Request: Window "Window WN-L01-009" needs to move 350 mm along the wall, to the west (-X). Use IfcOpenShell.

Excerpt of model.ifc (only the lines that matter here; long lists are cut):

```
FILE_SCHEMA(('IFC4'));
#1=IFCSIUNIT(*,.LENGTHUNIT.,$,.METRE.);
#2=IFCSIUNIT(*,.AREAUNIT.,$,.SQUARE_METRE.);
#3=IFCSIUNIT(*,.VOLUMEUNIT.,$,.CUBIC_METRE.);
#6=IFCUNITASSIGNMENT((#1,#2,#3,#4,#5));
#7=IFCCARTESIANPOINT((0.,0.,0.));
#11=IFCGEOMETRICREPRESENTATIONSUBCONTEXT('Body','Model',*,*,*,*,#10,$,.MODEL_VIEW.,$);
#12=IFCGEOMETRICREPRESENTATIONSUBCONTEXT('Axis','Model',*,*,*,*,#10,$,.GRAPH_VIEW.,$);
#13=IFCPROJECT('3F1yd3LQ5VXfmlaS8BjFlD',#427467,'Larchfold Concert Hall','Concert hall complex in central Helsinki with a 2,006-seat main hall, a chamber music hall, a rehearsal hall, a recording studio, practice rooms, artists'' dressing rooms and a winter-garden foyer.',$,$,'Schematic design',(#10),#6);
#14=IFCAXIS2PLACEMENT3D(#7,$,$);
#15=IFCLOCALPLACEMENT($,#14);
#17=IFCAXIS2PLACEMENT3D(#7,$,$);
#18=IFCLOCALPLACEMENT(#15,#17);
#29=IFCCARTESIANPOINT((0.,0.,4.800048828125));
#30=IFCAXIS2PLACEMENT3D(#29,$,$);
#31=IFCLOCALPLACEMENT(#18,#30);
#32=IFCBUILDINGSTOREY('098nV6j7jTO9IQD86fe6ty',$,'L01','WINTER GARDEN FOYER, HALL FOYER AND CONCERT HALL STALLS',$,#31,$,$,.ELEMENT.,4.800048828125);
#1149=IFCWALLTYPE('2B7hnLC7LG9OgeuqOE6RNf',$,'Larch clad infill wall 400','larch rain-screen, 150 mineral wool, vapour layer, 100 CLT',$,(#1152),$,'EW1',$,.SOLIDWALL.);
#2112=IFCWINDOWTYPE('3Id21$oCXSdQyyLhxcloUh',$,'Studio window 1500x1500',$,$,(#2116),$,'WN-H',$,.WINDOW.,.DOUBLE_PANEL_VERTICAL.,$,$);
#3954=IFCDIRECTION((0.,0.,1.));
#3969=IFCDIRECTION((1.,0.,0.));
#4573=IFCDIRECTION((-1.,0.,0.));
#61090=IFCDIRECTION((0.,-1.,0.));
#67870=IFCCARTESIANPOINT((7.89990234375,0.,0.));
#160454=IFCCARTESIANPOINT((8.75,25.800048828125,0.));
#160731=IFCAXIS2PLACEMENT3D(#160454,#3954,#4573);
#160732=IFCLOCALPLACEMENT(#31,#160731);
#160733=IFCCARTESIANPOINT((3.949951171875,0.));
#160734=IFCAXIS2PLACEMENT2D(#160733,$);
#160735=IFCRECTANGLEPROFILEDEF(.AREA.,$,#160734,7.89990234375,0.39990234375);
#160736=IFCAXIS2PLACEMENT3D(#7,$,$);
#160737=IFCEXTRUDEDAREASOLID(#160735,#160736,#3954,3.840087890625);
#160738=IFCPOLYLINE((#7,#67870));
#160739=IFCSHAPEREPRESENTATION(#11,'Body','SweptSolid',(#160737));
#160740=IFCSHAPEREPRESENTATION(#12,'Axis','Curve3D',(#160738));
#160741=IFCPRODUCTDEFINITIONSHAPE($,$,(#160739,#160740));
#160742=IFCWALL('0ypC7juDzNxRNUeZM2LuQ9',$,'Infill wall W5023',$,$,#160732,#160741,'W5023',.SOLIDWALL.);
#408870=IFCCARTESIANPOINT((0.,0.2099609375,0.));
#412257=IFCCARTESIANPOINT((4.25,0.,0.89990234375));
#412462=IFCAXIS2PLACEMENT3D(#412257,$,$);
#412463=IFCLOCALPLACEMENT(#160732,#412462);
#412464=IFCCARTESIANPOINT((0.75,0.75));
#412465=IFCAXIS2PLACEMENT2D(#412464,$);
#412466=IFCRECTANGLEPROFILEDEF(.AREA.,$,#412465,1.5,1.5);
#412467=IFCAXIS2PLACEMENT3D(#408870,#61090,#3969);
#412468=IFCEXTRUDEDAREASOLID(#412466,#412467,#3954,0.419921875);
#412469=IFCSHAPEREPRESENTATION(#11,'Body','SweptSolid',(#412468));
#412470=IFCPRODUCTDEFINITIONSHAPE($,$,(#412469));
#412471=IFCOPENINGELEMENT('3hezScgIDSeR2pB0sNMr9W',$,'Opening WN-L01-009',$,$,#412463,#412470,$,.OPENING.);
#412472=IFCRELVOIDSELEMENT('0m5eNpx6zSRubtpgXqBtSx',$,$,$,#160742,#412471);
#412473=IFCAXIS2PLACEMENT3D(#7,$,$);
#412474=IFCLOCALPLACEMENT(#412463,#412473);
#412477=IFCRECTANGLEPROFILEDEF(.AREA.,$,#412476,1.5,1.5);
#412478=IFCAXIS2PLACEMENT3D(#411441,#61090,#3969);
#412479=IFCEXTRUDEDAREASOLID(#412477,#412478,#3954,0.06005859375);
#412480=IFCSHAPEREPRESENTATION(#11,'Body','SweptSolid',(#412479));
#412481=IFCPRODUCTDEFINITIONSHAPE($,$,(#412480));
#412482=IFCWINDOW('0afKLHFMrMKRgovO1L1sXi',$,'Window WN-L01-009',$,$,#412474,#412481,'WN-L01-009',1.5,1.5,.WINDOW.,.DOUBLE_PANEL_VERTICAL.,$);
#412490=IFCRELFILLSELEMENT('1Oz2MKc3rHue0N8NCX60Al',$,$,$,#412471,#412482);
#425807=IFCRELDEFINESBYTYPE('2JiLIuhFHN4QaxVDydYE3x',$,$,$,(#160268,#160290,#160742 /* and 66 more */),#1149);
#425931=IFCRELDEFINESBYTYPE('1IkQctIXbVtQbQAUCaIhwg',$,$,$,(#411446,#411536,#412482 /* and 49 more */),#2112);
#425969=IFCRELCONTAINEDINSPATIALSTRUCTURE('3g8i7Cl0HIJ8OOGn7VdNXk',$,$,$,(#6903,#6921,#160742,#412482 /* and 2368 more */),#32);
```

```python
import ifcopenshell
import ifcopenshell.api.geometry
import ifcopenshell.util.placement
import ifcopenshell.util.unit

model = ifcopenshell.open("model.ifc")
unit_scale = ifcopenshell.util.unit.calculate_unit_scale(model)

window = model.by_id(412482)
opening = window.FillsVoids[0].RelatingOpeningElement
wall = opening.VoidsElements[0].RelatingBuildingElement

wall_matrix = ifcopenshell.util.placement.get_local_placement(wall.ObjectPlacement)
shift = wall_matrix[:3, 0] * 0.35 / unit_scale
before = ifcopenshell.util.placement.get_local_placement(window.ObjectPlacement)[:3, 3].copy()

# The window is placed relative to its opening, so it follows when the opening moves.
matrix = ifcopenshell.util.placement.get_local_placement(opening.ObjectPlacement)
matrix[:3, 3] += shift
ifcopenshell.api.geometry.edit_object_placement(
    model, product=opening, matrix=matrix, is_si=False, should_transform_children=True
)

after = ifcopenshell.util.placement.get_local_placement(window.ObjectPlacement)[:3, 3]
print("window moved by", (after - before).round(3) + 0.0)

model.write("model_updated.ifc")
```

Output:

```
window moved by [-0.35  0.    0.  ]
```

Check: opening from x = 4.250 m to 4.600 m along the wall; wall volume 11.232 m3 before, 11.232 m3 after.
